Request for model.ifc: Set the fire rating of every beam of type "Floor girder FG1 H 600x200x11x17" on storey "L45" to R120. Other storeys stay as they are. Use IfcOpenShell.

First a look at what the model holds.

```python
import ifcopenshell
import ifcopenshell.util.element

model = ifcopenshell.open("model.ifc")
print(model.schema)
storey = next(s for s in model.by_type("IfcBuildingStorey") if s.Name == "L45")
beams = [e for e in ifcopenshell.util.element.get_decomposition(storey) if e.is_a("IfcBeam")]
seen = {}
for e in beams:
    element_type = ifcopenshell.util.element.get_type(e)
    key = (element_type.Name if element_type != e and element_type else None, ifcopenshell.util.element.get_pset(e, "Pset_BeamCommon", "FireRating"))
    seen[key] = seen.get(key, 0) + 1
for (name, value), count in sorted(seen.items(), key=str):
    print(count, "x", name, "|", value)
```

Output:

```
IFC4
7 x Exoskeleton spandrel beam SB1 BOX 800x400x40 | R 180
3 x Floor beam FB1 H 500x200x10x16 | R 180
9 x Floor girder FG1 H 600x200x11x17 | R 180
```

```python
import ifcopenshell
import ifcopenshell.api.pset
import ifcopenshell.util.element

model = ifcopenshell.open("model.ifc")

storey = next(s for s in model.by_type("IfcBuildingStorey") if s.Name == "L45")
beams = [e for e in ifcopenshell.util.element.get_decomposition(storey) if e.is_a("IfcBeam")]

count = 0
for e in beams:
    element_type = ifcopenshell.util.element.get_type(e)
    if element_type in (None, e) or element_type.Name != "Floor girder FG1 H 600x200x11x17":
        continue
    # add_pset returns the element's existing set when there is one.
    pset = ifcopenshell.api.pset.add_pset(model, product=e, name="Pset_BeamCommon")
    ifcopenshell.api.pset.edit_pset(model, pset=pset, properties={"FireRating": "R120"})
    count += 1

print(count, "beams updated")

model.write("model_edited.ifc")
```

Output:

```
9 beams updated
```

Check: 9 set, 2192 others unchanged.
